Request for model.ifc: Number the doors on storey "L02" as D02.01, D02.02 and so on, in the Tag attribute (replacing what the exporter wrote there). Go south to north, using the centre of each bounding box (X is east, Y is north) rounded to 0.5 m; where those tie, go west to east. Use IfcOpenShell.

First a look at what the model holds.

```python
import ifcopenshell
import ifcopenshell.util.element
import ifcopenshell.util.placement

model = ifcopenshell.open("model.ifc")
print(model.schema)
storey = next(s for s in model.by_type("IfcBuildingStorey") if s.Name == "L02")
doors = [e for e in ifcopenshell.util.element.get_decomposition(storey) if e.is_a("IfcDoor")]
for e in sorted(doors, key=lambda e: e.id()):
    origin = ifcopenshell.util.placement.get_local_placement(e.ObjectPlacement)[:3, 3]
    print(e.id(), e.Tag, e.Name, origin.round(2) + 0.0, sep=" | ")
```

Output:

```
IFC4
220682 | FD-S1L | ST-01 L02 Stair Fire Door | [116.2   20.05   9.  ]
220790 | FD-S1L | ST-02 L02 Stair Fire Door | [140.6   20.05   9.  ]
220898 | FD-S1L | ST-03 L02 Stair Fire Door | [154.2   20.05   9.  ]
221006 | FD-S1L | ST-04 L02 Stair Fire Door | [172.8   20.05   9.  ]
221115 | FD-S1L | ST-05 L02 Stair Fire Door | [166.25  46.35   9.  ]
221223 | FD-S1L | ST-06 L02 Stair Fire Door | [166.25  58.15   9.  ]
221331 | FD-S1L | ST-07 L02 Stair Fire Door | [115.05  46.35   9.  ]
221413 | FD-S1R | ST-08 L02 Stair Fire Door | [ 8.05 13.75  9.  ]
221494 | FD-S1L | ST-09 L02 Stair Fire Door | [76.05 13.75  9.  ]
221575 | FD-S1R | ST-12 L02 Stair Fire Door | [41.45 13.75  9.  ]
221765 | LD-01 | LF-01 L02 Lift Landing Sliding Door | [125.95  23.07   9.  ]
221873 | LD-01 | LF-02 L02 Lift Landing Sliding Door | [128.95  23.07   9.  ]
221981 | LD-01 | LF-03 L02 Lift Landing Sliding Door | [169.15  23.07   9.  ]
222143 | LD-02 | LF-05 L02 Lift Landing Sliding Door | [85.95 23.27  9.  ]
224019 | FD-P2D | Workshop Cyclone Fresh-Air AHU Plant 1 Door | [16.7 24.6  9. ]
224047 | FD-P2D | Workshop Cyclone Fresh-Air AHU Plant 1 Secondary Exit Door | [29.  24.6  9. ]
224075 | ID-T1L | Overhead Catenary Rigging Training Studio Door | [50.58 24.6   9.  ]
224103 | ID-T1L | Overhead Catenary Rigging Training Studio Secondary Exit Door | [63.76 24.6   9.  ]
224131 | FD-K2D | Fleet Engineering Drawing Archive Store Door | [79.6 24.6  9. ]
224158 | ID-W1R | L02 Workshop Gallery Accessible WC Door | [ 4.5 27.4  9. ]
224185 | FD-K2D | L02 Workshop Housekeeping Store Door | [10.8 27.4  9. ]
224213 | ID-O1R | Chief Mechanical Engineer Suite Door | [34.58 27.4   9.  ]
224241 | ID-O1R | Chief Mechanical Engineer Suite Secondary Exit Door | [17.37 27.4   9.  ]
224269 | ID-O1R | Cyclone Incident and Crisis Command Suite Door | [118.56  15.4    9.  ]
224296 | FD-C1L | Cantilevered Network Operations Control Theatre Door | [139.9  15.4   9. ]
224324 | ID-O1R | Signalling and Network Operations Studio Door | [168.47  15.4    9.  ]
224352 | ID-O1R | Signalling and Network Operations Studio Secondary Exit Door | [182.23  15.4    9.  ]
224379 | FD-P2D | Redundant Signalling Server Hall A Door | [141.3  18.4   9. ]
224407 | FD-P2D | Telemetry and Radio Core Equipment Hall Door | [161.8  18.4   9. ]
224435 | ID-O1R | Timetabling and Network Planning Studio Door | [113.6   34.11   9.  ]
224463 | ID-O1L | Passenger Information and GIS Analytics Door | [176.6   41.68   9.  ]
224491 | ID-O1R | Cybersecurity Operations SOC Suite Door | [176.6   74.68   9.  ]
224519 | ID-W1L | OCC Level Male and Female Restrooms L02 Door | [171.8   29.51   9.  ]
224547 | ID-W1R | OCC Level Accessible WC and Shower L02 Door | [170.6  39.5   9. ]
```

```python
import ifcopenshell
import ifcopenshell.geom
import ifcopenshell.util.element
import ifcopenshell.util.shape

model = ifcopenshell.open("model.ifc")
settings = ifcopenshell.geom.settings()
settings.set("use-world-coords", True)


def centre(element):
    shape = ifcopenshell.geom.create_shape(settings, element)
    return ifcopenshell.util.shape.get_bbox_centroid(shape.geometry)


storey = next(s for s in model.by_type("IfcBuildingStorey") if s.Name == "L02")
doors = [e for e in ifcopenshell.util.element.get_decomposition(storey) if e.is_a("IfcDoor")]

# Insertion points can sit at a corner or the storey origin, so sort by the geometry (in metres).
centres = {e: centre(e) for e in doors}
doors.sort(key=lambda e: (round(centres[e][1] / 0.5), centres[e][0]))

for i, e in enumerate(doors, start=1):
    number = f"D02.{i:02d}"
    e.Tag = number
    print(e.id(), number)

model.write("model_rev.ifc")
```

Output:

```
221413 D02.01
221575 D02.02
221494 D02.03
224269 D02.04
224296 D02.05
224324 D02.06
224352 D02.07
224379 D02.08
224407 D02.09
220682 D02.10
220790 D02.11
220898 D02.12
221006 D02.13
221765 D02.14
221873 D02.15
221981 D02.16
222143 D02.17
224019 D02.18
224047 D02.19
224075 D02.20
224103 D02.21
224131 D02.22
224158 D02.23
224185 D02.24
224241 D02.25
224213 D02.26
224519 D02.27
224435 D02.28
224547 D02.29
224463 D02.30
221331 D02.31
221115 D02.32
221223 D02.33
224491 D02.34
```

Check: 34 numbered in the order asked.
